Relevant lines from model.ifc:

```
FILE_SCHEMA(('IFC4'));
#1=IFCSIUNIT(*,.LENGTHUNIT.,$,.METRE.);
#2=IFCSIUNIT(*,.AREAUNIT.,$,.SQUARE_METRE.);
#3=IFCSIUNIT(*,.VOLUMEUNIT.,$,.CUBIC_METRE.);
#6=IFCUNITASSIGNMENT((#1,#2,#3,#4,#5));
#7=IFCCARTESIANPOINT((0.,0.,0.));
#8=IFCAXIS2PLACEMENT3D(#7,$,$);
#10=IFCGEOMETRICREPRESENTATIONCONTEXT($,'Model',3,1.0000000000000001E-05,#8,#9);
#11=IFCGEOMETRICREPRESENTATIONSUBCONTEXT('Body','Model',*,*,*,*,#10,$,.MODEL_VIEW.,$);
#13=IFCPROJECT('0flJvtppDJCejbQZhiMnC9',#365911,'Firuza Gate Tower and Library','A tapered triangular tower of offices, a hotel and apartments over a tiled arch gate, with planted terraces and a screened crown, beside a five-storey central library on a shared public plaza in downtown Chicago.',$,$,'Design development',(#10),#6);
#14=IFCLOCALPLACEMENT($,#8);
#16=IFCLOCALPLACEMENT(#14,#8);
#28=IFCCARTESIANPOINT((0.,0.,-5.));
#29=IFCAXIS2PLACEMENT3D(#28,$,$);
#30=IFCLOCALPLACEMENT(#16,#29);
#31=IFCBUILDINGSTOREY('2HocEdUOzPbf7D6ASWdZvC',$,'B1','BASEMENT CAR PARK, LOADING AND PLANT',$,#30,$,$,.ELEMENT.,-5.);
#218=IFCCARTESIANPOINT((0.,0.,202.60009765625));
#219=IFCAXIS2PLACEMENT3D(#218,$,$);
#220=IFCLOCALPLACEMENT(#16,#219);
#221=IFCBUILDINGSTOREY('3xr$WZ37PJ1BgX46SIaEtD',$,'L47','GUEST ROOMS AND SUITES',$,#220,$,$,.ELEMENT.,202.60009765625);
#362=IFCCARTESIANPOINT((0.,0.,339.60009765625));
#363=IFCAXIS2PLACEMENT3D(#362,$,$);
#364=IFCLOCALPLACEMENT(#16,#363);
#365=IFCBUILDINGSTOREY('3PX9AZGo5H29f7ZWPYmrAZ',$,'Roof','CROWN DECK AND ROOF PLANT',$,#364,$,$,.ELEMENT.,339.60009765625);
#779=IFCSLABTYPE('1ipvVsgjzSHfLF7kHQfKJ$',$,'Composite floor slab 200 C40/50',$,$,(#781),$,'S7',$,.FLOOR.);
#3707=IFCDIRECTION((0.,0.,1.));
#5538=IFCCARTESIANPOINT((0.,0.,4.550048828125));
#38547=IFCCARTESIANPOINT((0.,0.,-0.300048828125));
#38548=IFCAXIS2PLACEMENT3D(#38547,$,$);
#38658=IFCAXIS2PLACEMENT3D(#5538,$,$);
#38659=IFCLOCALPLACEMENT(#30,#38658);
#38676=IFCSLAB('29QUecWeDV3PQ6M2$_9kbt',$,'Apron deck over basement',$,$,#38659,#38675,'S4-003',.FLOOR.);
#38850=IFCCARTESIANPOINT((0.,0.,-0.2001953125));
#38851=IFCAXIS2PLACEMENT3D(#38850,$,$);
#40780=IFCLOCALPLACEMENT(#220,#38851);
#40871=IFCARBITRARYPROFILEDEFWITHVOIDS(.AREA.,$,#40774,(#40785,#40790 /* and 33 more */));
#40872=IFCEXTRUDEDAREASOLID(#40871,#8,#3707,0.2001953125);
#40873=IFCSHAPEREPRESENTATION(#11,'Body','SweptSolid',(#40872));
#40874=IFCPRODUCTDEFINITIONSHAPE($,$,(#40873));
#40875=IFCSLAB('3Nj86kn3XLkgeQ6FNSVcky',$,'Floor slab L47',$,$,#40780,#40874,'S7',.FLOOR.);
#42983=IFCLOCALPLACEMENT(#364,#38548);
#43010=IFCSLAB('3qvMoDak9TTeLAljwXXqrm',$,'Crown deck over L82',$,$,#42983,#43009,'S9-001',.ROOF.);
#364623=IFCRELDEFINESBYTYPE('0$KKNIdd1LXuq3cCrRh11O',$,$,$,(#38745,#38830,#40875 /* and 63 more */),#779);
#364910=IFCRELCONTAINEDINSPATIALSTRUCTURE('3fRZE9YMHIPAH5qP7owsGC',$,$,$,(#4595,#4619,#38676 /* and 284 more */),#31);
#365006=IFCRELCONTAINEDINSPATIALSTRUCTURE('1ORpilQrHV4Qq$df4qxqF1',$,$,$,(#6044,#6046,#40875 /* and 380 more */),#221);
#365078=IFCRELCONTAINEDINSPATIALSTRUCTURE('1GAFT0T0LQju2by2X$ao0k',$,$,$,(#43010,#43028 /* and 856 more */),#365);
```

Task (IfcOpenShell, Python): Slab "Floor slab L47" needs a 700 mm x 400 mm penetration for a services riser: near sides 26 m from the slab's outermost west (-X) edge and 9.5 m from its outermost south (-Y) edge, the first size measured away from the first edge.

```python
import numpy as np
import ifcopenshell
import ifcopenshell.api.feature
import ifcopenshell.api.geometry
import ifcopenshell.api.root
import ifcopenshell.geom
import ifcopenshell.util.placement
import ifcopenshell.util.representation
import ifcopenshell.util.shape
import ifcopenshell.util.unit

model = ifcopenshell.open("model.ifc")
unit_scale = ifcopenshell.util.unit.calculate_unit_scale(model)
settings = ifcopenshell.geom.settings()


def volume(element):
    """Net volume in cubic metres, openings subtracted."""
    shape = ifcopenshell.geom.create_shape(settings, element)
    return ifcopenshell.util.shape.get_volume(shape.geometry)


slab = model.by_guid("3Nj86kn3XLkgeQ6FNSVcky")
before = volume(slab)

# Extent in the slab's own axes, in metres. The edges named are its -X and -Y sides.
slab_shape = ifcopenshell.geom.create_shape(settings, slab)
vertices = ifcopenshell.util.shape.get_vertices(slab_shape.geometry)
x_min, y_min, bottom = vertices.min(axis=0)
top = vertices[:, 2].max()

opening = ifcopenshell.api.root.create_entity(model, ifc_class="IfcOpeningElement", name="Services riser opening", predefined_type="OPENING")
context = ifcopenshell.util.representation.get_context(model, "Model", "Body", "MODEL_VIEW")
width, depth = 0.7, 0.4
outline = [(0.0, 0.0), (width, 0.0), (width, depth), (0.0, depth), (0.0, 0.0)]
# Overshoot both faces by 50 mm so the cut is clean.
shape = ifcopenshell.api.geometry.add_slab_representation(
    model, context=context, depth=top - bottom + 0.1, polyline=outline
)
ifcopenshell.api.geometry.assign_representation(model, product=opening, representation=shape)

matrix = ifcopenshell.util.placement.get_local_placement(slab.ObjectPlacement)
matrix[:, 3] = matrix @ np.append(np.array([x_min + 26, y_min + 9.5, bottom - 0.05]) / unit_scale, 1.0)
ifcopenshell.api.geometry.edit_object_placement(model, product=opening, matrix=matrix, is_si=False)
ifcopenshell.api.feature.add_feature(model, feature=opening, element=slab)

after = volume(slab)

print(f"slab volume {before:.3f} -> {after:.3f} m3")

model.write("model_v2.ifc")
```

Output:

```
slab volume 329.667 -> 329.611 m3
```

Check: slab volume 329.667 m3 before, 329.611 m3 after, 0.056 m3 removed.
